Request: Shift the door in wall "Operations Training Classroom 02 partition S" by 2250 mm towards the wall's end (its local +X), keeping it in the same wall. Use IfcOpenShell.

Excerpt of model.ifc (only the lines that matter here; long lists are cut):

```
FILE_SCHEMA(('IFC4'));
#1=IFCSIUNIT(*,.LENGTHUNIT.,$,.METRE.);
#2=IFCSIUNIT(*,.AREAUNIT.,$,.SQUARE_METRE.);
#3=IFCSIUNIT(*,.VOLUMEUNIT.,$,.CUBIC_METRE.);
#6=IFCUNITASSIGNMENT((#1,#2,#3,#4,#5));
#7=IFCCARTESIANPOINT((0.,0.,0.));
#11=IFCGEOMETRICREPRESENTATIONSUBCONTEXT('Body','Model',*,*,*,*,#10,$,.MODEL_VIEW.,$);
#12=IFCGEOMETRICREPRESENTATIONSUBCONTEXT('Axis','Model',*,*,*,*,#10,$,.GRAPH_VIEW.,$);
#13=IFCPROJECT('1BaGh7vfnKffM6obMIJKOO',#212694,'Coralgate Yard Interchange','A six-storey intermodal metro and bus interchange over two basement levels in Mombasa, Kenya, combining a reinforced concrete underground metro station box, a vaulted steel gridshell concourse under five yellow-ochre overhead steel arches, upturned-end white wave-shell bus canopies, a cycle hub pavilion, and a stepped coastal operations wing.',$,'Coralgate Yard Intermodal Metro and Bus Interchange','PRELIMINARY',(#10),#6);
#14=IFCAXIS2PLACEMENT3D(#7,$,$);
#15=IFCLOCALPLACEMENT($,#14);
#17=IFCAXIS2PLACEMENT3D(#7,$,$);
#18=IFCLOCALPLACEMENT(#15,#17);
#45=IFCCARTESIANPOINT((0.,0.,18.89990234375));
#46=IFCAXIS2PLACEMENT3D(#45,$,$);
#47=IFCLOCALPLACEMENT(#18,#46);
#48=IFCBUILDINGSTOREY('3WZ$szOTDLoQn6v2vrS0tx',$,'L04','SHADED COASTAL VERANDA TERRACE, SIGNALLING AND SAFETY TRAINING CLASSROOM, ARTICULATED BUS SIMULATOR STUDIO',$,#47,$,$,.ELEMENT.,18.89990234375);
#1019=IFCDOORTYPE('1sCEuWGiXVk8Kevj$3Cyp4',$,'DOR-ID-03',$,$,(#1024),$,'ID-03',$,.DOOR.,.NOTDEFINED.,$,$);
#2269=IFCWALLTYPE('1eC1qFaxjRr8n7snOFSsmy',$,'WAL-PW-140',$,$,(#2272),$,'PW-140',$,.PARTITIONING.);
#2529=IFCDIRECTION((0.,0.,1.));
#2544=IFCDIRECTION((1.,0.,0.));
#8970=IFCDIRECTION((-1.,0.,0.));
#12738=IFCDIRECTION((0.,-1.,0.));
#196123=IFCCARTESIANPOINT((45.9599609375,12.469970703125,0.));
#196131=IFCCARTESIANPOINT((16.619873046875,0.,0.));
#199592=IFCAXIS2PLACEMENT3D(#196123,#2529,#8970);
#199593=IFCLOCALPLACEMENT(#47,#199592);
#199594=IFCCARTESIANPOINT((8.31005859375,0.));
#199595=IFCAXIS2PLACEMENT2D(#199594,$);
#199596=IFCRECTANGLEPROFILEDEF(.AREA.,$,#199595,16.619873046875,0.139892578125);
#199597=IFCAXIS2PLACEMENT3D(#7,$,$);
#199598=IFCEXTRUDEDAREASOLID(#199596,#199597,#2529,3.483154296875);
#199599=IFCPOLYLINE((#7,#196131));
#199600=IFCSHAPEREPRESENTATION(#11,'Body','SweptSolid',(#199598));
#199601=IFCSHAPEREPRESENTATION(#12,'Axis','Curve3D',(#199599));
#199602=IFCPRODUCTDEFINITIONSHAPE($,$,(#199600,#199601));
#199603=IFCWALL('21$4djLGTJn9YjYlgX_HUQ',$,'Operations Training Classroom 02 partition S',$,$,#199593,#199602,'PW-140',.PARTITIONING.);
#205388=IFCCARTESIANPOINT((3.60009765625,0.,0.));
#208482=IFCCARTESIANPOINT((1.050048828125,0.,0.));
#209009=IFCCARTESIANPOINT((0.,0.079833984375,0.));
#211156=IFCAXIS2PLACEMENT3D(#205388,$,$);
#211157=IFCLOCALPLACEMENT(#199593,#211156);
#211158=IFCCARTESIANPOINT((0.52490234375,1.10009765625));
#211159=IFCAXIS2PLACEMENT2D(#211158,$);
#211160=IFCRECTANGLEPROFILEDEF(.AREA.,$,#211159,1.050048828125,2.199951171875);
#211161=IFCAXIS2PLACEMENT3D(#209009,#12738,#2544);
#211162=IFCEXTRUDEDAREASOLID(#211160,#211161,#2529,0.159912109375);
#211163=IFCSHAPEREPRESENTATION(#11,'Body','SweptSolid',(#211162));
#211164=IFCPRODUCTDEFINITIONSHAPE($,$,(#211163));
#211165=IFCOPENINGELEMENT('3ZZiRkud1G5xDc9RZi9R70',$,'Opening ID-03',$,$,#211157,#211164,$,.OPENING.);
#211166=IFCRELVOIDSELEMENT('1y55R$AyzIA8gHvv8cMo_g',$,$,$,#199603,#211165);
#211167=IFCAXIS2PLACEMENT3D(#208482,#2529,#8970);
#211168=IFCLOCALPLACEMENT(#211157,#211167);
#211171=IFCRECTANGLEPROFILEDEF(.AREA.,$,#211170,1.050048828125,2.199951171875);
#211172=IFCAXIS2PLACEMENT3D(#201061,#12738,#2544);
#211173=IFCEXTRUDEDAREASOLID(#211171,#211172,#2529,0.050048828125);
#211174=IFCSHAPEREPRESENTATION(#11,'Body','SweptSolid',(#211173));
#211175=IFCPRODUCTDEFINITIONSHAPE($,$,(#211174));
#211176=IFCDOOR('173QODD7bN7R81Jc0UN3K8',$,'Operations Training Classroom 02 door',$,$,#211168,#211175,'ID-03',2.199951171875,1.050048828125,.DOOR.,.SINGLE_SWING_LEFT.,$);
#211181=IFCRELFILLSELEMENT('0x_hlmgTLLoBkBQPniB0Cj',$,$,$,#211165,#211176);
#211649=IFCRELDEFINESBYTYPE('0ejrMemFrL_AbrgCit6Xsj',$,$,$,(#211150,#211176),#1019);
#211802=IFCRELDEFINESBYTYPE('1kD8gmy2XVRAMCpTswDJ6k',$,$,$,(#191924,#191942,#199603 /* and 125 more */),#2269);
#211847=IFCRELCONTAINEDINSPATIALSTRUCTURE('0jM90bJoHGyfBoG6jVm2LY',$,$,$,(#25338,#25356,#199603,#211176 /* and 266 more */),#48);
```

```python
import ifcopenshell
import ifcopenshell.api.geometry
import ifcopenshell.util.placement
import ifcopenshell.util.unit

model = ifcopenshell.open("model.ifc")
unit_scale = ifcopenshell.util.unit.calculate_unit_scale(model)

door = model.by_guid("173QODD7bN7R81Jc0UN3K8")
opening = door.FillsVoids[0].RelatingOpeningElement
wall = opening.VoidsElements[0].RelatingBuildingElement

wall_matrix = ifcopenshell.util.placement.get_local_placement(wall.ObjectPlacement)
shift = wall_matrix[:3, 0] * 2.25 / unit_scale
before = ifcopenshell.util.placement.get_local_placement(door.ObjectPlacement)[:3, 3].copy()

# The door is placed relative to its opening, so it follows when the opening moves.
matrix = ifcopenshell.util.placement.get_local_placement(opening.ObjectPlacement)
matrix[:3, 3] += shift
ifcopenshell.api.geometry.edit_object_placement(
    model, product=opening, matrix=matrix, is_si=False, should_transform_children=True
)

after = ifcopenshell.util.placement.get_local_placement(door.ObjectPlacement)[:3, 3]
print("door moved by", (after - before).round(3) + 0.0)

model.write("model_edited.ifc")
```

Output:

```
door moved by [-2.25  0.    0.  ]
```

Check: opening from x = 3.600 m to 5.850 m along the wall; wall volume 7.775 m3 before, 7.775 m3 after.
